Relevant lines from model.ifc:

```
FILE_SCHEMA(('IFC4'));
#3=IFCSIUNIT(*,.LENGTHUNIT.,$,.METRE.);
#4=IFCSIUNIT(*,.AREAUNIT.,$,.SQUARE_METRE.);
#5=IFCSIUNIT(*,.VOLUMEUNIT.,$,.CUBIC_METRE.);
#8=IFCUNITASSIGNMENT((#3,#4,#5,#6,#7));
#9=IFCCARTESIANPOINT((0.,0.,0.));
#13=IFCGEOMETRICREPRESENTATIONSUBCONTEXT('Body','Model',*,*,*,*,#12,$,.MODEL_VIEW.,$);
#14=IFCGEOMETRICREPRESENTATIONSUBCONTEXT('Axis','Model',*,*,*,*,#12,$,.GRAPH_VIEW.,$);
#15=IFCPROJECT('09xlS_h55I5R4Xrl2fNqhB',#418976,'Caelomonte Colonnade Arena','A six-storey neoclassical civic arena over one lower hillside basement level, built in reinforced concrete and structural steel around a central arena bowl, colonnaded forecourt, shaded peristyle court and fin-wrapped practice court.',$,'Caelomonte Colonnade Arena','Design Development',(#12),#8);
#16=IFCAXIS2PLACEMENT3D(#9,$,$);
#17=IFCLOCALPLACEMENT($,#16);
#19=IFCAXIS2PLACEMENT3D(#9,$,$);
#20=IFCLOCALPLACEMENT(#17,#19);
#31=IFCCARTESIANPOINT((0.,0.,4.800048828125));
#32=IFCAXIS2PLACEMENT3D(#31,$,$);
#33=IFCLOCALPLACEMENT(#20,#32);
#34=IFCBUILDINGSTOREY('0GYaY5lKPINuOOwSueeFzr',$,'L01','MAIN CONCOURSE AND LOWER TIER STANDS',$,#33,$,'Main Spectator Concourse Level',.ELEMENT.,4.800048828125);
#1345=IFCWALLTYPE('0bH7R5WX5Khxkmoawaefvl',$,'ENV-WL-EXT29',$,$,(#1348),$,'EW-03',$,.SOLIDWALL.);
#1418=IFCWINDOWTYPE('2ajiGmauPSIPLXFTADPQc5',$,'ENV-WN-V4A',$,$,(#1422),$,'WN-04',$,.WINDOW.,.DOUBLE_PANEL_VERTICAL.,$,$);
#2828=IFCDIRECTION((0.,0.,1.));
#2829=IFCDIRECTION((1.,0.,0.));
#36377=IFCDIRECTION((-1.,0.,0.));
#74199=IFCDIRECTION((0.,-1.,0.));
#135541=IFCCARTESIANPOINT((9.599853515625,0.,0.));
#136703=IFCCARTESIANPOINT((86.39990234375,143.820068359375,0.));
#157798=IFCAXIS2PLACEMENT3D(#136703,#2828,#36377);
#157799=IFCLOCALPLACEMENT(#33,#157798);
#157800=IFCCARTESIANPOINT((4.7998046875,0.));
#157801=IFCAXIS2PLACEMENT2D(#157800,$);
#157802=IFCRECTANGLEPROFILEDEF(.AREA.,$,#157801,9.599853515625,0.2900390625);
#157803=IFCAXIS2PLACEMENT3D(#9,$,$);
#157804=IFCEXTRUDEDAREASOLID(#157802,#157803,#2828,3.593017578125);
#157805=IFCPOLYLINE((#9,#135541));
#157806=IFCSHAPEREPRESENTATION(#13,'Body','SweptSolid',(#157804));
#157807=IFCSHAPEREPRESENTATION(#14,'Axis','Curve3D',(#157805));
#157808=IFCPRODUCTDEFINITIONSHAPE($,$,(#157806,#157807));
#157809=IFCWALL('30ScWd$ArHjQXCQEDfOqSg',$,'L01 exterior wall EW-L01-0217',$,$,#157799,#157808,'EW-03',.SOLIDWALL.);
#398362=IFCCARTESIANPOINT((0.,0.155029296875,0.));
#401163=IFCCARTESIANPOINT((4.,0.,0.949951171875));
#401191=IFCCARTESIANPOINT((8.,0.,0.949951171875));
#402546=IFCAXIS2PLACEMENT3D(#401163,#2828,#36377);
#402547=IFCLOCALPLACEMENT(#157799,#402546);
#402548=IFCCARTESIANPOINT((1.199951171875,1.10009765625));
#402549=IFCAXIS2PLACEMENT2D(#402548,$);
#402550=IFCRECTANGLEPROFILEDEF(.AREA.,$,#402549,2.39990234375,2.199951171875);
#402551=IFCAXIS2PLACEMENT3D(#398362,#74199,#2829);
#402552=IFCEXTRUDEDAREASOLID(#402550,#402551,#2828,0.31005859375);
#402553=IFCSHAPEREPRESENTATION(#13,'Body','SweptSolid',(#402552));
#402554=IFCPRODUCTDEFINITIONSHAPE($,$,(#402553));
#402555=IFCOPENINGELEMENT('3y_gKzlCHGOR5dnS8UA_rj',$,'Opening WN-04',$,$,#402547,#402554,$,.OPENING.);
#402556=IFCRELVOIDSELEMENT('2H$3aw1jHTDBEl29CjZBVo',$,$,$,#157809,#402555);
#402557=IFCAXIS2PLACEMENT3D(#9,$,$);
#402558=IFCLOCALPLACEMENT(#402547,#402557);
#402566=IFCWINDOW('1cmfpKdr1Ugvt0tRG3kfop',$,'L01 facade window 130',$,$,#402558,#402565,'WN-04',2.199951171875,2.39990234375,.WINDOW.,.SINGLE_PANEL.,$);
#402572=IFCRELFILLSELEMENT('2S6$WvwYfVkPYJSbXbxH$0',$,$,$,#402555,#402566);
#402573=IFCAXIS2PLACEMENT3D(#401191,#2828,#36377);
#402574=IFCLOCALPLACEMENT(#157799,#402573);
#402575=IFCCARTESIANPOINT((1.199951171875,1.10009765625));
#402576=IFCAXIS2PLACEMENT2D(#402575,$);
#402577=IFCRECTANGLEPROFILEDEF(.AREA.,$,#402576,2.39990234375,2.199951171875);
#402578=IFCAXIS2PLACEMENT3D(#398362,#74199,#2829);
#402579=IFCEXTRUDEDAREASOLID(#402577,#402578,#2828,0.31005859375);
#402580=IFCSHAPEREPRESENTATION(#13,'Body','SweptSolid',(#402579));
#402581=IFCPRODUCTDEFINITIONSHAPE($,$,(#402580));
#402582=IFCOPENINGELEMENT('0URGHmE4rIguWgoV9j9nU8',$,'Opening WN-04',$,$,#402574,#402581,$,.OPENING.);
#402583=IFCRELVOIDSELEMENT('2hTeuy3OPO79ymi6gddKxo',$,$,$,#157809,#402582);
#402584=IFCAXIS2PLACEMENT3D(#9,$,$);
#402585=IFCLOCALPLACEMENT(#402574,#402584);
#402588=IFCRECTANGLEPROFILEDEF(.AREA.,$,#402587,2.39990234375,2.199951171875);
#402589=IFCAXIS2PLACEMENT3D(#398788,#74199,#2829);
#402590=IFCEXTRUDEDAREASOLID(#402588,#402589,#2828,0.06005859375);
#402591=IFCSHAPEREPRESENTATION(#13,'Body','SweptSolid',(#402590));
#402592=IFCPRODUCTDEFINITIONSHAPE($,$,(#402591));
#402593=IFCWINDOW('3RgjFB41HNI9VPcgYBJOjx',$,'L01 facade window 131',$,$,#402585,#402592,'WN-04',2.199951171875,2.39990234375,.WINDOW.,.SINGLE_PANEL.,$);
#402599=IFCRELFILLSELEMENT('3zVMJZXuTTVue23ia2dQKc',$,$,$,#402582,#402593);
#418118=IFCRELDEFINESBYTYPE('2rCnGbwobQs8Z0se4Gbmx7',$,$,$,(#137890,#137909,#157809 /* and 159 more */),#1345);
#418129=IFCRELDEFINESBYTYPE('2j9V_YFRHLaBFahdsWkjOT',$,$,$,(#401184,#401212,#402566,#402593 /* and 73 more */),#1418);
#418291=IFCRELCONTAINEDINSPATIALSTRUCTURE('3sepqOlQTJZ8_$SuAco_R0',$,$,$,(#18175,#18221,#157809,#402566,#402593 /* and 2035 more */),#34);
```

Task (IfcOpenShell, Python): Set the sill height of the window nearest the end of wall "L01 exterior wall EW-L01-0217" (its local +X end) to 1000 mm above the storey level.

```python
import numpy as np
import ifcopenshell
import ifcopenshell.api.geometry
import ifcopenshell.geom
import ifcopenshell.util.element
import ifcopenshell.util.placement
import ifcopenshell.util.shape
import ifcopenshell.util.unit

model = ifcopenshell.open("model.ifc")
unit_scale = ifcopenshell.util.unit.calculate_unit_scale(model)

window = model.by_guid("3RgjFB41HNI9VPcgYBJOjx")
opening = window.FillsVoids[0].RelatingOpeningElement
storey = ifcopenshell.util.element.get_container(window, ifc_class="IfcBuildingStorey")
level = ifcopenshell.util.placement.get_local_placement(storey.ObjectPlacement)[2, 3]

# The opening's origin need not be at the sill, so measure its lowest point.
shape = ifcopenshell.geom.create_shape(ifcopenshell.geom.settings(), opening)
bottom = ifcopenshell.util.shape.get_shape_bottom_elevation(shape, shape.geometry) / unit_scale
dz = level + 1.0 - bottom

shift = np.array([0.0, 0.0, dz])
# The window is placed relative to its opening, so it follows when the opening moves.
matrix = ifcopenshell.util.placement.get_local_placement(opening.ObjectPlacement)
matrix[:3, 3] += shift
ifcopenshell.api.geometry.edit_object_placement(
    model, product=opening, matrix=matrix, is_si=False, should_transform_children=True
)

print(f"moved by {dz * unit_scale:+.3f} m")

model.write("model_v2.ifc")
```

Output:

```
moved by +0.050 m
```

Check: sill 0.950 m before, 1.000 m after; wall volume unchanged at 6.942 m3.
